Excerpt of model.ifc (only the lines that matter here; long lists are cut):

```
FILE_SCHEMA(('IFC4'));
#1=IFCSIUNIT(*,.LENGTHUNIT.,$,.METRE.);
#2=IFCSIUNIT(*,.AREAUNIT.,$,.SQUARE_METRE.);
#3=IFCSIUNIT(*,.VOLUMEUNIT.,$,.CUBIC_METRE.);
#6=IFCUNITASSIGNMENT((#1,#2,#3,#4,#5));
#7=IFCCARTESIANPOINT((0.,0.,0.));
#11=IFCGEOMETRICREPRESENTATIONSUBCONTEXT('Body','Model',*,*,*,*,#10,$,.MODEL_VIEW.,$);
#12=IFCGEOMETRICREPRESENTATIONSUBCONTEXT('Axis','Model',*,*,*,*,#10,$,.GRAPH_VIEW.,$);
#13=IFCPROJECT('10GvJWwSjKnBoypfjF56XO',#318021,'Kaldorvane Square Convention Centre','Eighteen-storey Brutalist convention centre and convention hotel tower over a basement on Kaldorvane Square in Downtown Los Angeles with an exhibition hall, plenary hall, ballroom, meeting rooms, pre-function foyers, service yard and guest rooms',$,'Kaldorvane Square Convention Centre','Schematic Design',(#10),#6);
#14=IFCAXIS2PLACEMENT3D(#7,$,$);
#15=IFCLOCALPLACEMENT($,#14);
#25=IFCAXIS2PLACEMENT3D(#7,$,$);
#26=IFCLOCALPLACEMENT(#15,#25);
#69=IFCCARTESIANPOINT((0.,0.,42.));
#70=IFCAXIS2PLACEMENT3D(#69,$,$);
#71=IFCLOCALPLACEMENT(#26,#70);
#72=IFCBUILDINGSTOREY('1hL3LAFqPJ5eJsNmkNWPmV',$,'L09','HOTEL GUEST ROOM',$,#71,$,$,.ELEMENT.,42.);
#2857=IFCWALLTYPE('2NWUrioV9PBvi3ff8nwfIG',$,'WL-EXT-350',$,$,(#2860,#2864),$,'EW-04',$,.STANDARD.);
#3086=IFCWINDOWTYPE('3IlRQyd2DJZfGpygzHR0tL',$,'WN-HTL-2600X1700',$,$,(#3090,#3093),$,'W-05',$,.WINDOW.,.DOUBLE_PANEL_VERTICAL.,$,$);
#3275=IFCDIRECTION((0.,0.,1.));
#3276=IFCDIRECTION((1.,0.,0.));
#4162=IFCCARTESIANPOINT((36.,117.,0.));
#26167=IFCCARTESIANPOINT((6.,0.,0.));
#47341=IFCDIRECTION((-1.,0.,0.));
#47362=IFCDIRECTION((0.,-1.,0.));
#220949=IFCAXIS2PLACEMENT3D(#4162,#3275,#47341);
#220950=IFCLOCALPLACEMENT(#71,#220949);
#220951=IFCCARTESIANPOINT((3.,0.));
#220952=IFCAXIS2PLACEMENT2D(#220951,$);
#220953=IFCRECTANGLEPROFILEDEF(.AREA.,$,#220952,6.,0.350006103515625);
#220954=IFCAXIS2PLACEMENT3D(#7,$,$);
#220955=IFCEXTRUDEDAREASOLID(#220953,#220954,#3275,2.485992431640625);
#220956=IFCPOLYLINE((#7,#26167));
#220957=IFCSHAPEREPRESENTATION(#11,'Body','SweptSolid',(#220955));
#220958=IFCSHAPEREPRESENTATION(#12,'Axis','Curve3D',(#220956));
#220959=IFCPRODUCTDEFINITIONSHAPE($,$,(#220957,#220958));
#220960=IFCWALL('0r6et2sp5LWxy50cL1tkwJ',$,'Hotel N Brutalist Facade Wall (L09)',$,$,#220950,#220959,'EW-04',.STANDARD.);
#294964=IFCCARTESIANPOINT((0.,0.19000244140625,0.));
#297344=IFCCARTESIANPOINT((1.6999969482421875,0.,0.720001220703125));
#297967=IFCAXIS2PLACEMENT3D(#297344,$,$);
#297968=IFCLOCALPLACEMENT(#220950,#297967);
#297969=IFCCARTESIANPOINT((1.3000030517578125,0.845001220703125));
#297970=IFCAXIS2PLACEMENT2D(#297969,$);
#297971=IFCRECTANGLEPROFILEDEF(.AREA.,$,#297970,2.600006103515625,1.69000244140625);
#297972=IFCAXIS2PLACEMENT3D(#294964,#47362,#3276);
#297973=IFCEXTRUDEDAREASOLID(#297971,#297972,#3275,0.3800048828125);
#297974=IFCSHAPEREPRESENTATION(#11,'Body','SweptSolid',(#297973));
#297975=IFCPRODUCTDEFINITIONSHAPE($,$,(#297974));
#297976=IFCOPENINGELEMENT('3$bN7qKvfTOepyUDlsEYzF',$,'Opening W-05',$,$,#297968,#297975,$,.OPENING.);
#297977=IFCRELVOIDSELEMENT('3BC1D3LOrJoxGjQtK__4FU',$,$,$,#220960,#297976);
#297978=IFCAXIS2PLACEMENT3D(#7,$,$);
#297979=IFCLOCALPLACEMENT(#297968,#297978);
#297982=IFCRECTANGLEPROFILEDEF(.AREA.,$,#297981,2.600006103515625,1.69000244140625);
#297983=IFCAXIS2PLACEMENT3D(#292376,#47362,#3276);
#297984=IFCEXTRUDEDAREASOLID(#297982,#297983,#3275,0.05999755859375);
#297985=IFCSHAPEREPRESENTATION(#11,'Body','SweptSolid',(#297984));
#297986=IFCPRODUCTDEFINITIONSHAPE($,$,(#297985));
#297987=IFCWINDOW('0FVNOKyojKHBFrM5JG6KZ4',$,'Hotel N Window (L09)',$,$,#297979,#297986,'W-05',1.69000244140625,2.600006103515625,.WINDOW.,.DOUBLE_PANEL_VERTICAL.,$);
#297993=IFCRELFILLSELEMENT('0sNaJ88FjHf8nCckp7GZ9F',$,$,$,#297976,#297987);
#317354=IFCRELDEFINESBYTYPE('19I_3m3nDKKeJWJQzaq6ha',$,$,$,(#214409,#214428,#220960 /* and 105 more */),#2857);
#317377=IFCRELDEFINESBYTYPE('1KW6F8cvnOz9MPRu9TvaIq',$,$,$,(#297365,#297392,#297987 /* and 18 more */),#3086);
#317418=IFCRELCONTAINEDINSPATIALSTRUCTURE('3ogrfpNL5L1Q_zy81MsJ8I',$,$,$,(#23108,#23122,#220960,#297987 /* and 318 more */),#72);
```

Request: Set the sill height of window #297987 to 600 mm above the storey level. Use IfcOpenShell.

```python
import numpy as np
import ifcopenshell
import ifcopenshell.api.geometry
import ifcopenshell.geom
import ifcopenshell.util.element
import ifcopenshell.util.placement
import ifcopenshell.util.shape
import ifcopenshell.util.unit

model = ifcopenshell.open("model.ifc")
unit_scale = ifcopenshell.util.unit.calculate_unit_scale(model)

window = model.by_guid("0FVNOKyojKHBFrM5JG6KZ4")
opening = window.FillsVoids[0].RelatingOpeningElement
storey = ifcopenshell.util.element.get_container(window, ifc_class="IfcBuildingStorey")
level = ifcopenshell.util.placement.get_local_placement(storey.ObjectPlacement)[2, 3]

# The opening's origin need not be at the sill, so measure its lowest point.
shape = ifcopenshell.geom.create_shape(ifcopenshell.geom.settings(), opening)
bottom = ifcopenshell.util.shape.get_shape_bottom_elevation(shape, shape.geometry) / unit_scale
dz = level + 0.6 / unit_scale - bottom

shift = np.array([0.0, 0.0, dz])
# The window is placed relative to its opening, so it follows when the opening moves.
matrix = ifcopenshell.util.placement.get_local_placement(opening.ObjectPlacement)
matrix[:3, 3] += shift
ifcopenshell.api.geometry.edit_object_placement(
    model, product=opening, matrix=matrix, is_si=False, should_transform_children=True
)

print(f"moved by {dz * unit_scale:+.3f} m")

model.write("model_edited.ifc")
```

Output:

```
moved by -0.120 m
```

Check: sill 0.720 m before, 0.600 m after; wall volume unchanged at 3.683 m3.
